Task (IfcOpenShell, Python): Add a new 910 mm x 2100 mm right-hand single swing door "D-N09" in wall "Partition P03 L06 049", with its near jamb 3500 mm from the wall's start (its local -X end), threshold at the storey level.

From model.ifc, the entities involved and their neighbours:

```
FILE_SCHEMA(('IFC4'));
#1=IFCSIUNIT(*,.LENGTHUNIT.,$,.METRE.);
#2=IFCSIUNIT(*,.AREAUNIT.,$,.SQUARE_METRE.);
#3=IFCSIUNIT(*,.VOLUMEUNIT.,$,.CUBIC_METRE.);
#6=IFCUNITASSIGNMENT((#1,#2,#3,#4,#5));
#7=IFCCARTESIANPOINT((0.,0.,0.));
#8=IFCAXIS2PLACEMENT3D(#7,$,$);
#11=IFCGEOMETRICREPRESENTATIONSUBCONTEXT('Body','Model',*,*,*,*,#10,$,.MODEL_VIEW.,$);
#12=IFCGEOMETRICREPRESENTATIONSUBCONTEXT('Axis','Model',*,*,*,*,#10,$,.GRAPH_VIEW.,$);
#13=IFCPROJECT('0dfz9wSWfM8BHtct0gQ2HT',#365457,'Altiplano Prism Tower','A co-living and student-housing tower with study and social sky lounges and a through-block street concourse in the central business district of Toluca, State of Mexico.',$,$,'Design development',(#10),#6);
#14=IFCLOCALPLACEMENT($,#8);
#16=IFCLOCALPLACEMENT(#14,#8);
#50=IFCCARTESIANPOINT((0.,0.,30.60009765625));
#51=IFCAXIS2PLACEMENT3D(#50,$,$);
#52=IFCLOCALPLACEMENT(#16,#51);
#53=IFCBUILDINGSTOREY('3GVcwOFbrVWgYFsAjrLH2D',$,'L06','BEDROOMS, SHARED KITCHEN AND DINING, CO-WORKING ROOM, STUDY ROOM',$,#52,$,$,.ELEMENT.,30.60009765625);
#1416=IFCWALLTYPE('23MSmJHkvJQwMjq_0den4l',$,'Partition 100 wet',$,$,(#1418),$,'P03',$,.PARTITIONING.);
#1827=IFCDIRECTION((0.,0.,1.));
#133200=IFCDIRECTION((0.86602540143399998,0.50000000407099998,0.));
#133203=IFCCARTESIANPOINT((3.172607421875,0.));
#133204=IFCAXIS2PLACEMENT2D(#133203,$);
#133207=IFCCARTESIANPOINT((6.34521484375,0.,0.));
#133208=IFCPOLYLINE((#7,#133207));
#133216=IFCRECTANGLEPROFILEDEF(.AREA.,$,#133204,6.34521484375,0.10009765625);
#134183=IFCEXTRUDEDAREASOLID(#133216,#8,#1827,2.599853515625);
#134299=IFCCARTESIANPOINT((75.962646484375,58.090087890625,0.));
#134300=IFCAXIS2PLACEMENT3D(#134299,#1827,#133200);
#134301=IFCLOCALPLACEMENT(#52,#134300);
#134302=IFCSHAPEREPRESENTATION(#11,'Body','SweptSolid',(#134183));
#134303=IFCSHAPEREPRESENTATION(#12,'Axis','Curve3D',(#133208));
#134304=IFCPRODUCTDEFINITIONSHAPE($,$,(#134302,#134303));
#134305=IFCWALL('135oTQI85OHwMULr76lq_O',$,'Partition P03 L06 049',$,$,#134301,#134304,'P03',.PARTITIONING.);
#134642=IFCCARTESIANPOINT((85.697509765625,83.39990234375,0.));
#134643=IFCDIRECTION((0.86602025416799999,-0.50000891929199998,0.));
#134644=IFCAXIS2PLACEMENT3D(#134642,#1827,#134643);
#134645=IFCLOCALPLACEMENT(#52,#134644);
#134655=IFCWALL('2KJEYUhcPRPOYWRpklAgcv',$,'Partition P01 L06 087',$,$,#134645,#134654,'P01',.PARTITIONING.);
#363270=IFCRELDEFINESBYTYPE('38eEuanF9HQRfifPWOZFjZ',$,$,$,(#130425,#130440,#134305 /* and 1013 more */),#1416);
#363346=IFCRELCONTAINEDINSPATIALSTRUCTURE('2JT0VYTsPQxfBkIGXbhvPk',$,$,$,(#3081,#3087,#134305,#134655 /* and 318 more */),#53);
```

```python
import numpy as np
import ifcopenshell
import ifcopenshell.api.feature
import ifcopenshell.api.geometry
import ifcopenshell.api.root
import ifcopenshell.api.spatial
import ifcopenshell.geom
import ifcopenshell.util.element
import ifcopenshell.util.placement
import ifcopenshell.util.representation
import ifcopenshell.util.shape
import ifcopenshell.util.unit

model = ifcopenshell.open("model.ifc")
unit_scale = ifcopenshell.util.unit.calculate_unit_scale(model)
settings = ifcopenshell.geom.settings()


def volume(element):
    """Net volume in cubic metres, openings subtracted."""
    shape = ifcopenshell.geom.create_shape(settings, element)
    return ifcopenshell.util.shape.get_volume(shape.geometry)


wall = model.by_guid("135oTQI85OHwMULr76lq_O")
storey = ifcopenshell.util.element.get_container(wall, ifc_class="IfcBuildingStorey")
context = ifcopenshell.util.representation.get_context(model, "Model", "Body", "MODEL_VIEW")
before = volume(wall)

width, height, from_end, sill = 0.91, 2.1, 3.5, 0.0  # metres

# The wall runs along its own X axis, and the end named is its -X end.
wall_shape = ifcopenshell.geom.create_shape(settings, wall)
x, y, z = ifcopenshell.util.shape.get_vertices(wall_shape.geometry).T
start = x.min() + from_end
face, thickness = float(y.min()), float(y.max() - y.min())
wall_matrix = ifcopenshell.util.placement.get_local_placement(wall.ObjectPlacement)
level = ifcopenshell.util.placement.get_local_placement(storey.ObjectPlacement)[2, 3]


def in_wall(x, y):
    """Placement at x, y metres in the wall's axes, at sill height."""
    matrix = wall_matrix.copy()
    matrix[:, 3] = wall_matrix @ np.array([x / unit_scale, y / unit_scale, 0.0, 1.0])
    matrix[2, 3] = level + sill / unit_scale
    return matrix


# Opening: a box that overshoots both wall faces by 50 mm.
opening = ifcopenshell.api.root.create_entity(model, ifc_class="IfcOpeningElement", predefined_type="OPENING")
box = ifcopenshell.api.geometry.add_wall_representation(
    model, context=context, length=width, height=height, thickness=thickness + 0.1
)
ifcopenshell.api.geometry.assign_representation(model, product=opening, representation=box)
ifcopenshell.api.geometry.edit_object_placement(model, product=opening, matrix=in_wall(start, face - 0.05), is_si=False)
ifcopenshell.api.feature.add_feature(model, feature=opening, element=wall)

door = ifcopenshell.api.root.create_entity(model, ifc_class="IfcDoor", name="D-N09", predefined_type="DOOR")
door.OverallWidth, door.OverallHeight = width / unit_scale, height / unit_scale
door.OperationType = "SINGLE_SWING_RIGHT"
body = ifcopenshell.api.geometry.add_door_representation(
    model,
    context=context,
    overall_width=door.OverallWidth,
    overall_height=door.OverallHeight,
    operation_type="SINGLE_SWING_RIGHT",
    lining_properties={"LiningDepth": thickness / unit_scale, "ThresholdDepth": thickness / unit_scale},
)
ifcopenshell.api.geometry.assign_representation(model, product=door, representation=body)
ifcopenshell.api.spatial.assign_container(model, products=[door], relating_structure=storey)
ifcopenshell.api.feature.add_filling(model, opening=opening, element=door)

# The lining spans the wall, so the door starts at the wall face.
ifcopenshell.api.geometry.edit_object_placement(model, product=door, matrix=in_wall(start, face), is_si=False)

after = volume(wall)

print(f"wall volume {before:.3f} -> {after:.3f} m3")

model.write("model_rev.ifc")
```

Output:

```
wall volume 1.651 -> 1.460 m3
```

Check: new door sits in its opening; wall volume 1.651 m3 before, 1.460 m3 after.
